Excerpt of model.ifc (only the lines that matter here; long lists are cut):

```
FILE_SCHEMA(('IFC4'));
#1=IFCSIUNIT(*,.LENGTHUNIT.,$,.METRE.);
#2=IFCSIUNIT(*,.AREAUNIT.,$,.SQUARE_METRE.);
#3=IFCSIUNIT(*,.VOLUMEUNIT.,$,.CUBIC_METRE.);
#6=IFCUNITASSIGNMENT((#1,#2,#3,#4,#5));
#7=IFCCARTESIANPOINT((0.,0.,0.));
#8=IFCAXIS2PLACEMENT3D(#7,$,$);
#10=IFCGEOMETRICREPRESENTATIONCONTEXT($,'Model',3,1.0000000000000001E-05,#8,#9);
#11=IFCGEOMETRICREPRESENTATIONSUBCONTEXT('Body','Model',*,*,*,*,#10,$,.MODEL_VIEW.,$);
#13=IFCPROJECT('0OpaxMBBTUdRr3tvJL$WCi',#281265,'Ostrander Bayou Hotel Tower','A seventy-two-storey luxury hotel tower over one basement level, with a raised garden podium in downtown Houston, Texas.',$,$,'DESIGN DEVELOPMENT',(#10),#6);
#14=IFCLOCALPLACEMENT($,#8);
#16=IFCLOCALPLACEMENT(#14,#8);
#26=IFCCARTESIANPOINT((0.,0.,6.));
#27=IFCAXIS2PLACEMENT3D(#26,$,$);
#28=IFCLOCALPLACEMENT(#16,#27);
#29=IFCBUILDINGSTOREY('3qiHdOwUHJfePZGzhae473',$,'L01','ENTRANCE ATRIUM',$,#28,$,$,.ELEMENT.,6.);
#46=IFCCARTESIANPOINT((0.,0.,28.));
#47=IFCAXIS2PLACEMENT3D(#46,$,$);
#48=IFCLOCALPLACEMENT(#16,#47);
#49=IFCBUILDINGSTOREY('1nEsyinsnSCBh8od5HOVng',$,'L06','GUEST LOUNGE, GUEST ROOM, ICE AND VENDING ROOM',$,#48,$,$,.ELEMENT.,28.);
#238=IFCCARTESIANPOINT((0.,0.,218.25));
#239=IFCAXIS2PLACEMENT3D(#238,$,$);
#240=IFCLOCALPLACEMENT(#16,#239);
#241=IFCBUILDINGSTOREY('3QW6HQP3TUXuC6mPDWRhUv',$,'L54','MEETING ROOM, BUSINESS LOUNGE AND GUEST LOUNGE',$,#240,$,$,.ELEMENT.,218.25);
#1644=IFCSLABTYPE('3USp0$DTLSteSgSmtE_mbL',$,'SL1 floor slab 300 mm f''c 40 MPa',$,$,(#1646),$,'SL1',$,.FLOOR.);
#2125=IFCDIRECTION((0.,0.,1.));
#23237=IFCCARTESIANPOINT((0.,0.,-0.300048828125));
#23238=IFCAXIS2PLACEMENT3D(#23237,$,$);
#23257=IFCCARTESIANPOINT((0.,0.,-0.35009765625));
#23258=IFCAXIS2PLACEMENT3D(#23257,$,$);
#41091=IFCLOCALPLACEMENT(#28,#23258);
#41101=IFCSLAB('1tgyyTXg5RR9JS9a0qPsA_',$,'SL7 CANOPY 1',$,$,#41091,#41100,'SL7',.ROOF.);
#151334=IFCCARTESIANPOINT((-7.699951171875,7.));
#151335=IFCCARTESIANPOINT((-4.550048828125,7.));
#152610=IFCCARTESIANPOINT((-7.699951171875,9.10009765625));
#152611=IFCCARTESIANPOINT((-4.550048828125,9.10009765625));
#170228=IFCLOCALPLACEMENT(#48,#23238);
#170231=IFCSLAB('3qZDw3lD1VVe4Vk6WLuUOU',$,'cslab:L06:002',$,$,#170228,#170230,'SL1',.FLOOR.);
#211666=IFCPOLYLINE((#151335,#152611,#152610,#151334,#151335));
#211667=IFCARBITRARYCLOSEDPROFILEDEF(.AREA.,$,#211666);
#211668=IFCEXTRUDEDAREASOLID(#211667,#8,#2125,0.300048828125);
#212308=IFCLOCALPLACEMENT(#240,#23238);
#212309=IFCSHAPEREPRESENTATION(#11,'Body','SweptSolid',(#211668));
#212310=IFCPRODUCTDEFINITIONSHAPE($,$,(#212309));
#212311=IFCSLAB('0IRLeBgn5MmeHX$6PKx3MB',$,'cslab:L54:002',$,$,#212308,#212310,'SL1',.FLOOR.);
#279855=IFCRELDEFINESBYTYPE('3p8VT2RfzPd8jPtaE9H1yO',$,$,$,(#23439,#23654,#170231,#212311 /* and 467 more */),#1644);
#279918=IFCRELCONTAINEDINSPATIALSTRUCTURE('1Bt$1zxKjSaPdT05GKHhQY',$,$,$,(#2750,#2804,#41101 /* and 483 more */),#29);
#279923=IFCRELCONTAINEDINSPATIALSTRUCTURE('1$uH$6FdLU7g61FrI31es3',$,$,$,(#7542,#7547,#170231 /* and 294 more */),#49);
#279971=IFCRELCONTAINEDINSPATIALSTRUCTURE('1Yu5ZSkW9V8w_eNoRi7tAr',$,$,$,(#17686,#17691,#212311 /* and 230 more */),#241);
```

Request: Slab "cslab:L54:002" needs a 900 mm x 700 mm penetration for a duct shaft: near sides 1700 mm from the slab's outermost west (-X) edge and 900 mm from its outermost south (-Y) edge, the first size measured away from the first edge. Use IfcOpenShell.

```python
import numpy as np
import ifcopenshell
import ifcopenshell.api.feature
import ifcopenshell.api.geometry
import ifcopenshell.api.root
import ifcopenshell.geom
import ifcopenshell.util.placement
import ifcopenshell.util.representation
import ifcopenshell.util.shape
import ifcopenshell.util.unit

model = ifcopenshell.open("model.ifc")
unit_scale = ifcopenshell.util.unit.calculate_unit_scale(model)
settings = ifcopenshell.geom.settings()


def volume(element):
    """Net volume in cubic metres, openings subtracted."""
    shape = ifcopenshell.geom.create_shape(settings, element)
    return ifcopenshell.util.shape.get_volume(shape.geometry)


slab = model.by_guid("0IRLeBgn5MmeHX$6PKx3MB")
before = volume(slab)

# Extent in the slab's own axes, in metres. The edges named are its -X and -Y sides.
slab_shape = ifcopenshell.geom.create_shape(settings, slab)
vertices = ifcopenshell.util.shape.get_vertices(slab_shape.geometry)
x_min, y_min, bottom = vertices.min(axis=0)
top = vertices[:, 2].max()

opening = ifcopenshell.api.root.create_entity(model, ifc_class="IfcOpeningElement", name="Duct shaft opening", predefined_type="OPENING")
context = ifcopenshell.util.representation.get_context(model, "Model", "Body", "MODEL_VIEW")
width, depth = 0.9, 0.7
outline = [(0.0, 0.0), (width, 0.0), (width, depth), (0.0, depth), (0.0, 0.0)]
# Overshoot both faces by 50 mm so the cut is clean.
shape = ifcopenshell.api.geometry.add_slab_representation(
    model, context=context, depth=top - bottom + 0.1, polyline=outline
)
ifcopenshell.api.geometry.assign_representation(model, product=opening, representation=shape)

matrix = ifcopenshell.util.placement.get_local_placement(slab.ObjectPlacement)
matrix[:, 3] = matrix @ np.append(np.array([x_min + 1.7, y_min + 0.9, bottom - 0.05]) / unit_scale, 1.0)
ifcopenshell.api.geometry.edit_object_placement(model, product=opening, matrix=matrix, is_si=False)
ifcopenshell.api.feature.add_feature(model, feature=opening, element=slab)

after = volume(slab)

print(f"slab volume {before:.3f} -> {after:.3f} m3")

model.write("model_v2.ifc")
```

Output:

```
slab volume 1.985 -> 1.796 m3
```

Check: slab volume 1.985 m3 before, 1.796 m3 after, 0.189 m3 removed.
